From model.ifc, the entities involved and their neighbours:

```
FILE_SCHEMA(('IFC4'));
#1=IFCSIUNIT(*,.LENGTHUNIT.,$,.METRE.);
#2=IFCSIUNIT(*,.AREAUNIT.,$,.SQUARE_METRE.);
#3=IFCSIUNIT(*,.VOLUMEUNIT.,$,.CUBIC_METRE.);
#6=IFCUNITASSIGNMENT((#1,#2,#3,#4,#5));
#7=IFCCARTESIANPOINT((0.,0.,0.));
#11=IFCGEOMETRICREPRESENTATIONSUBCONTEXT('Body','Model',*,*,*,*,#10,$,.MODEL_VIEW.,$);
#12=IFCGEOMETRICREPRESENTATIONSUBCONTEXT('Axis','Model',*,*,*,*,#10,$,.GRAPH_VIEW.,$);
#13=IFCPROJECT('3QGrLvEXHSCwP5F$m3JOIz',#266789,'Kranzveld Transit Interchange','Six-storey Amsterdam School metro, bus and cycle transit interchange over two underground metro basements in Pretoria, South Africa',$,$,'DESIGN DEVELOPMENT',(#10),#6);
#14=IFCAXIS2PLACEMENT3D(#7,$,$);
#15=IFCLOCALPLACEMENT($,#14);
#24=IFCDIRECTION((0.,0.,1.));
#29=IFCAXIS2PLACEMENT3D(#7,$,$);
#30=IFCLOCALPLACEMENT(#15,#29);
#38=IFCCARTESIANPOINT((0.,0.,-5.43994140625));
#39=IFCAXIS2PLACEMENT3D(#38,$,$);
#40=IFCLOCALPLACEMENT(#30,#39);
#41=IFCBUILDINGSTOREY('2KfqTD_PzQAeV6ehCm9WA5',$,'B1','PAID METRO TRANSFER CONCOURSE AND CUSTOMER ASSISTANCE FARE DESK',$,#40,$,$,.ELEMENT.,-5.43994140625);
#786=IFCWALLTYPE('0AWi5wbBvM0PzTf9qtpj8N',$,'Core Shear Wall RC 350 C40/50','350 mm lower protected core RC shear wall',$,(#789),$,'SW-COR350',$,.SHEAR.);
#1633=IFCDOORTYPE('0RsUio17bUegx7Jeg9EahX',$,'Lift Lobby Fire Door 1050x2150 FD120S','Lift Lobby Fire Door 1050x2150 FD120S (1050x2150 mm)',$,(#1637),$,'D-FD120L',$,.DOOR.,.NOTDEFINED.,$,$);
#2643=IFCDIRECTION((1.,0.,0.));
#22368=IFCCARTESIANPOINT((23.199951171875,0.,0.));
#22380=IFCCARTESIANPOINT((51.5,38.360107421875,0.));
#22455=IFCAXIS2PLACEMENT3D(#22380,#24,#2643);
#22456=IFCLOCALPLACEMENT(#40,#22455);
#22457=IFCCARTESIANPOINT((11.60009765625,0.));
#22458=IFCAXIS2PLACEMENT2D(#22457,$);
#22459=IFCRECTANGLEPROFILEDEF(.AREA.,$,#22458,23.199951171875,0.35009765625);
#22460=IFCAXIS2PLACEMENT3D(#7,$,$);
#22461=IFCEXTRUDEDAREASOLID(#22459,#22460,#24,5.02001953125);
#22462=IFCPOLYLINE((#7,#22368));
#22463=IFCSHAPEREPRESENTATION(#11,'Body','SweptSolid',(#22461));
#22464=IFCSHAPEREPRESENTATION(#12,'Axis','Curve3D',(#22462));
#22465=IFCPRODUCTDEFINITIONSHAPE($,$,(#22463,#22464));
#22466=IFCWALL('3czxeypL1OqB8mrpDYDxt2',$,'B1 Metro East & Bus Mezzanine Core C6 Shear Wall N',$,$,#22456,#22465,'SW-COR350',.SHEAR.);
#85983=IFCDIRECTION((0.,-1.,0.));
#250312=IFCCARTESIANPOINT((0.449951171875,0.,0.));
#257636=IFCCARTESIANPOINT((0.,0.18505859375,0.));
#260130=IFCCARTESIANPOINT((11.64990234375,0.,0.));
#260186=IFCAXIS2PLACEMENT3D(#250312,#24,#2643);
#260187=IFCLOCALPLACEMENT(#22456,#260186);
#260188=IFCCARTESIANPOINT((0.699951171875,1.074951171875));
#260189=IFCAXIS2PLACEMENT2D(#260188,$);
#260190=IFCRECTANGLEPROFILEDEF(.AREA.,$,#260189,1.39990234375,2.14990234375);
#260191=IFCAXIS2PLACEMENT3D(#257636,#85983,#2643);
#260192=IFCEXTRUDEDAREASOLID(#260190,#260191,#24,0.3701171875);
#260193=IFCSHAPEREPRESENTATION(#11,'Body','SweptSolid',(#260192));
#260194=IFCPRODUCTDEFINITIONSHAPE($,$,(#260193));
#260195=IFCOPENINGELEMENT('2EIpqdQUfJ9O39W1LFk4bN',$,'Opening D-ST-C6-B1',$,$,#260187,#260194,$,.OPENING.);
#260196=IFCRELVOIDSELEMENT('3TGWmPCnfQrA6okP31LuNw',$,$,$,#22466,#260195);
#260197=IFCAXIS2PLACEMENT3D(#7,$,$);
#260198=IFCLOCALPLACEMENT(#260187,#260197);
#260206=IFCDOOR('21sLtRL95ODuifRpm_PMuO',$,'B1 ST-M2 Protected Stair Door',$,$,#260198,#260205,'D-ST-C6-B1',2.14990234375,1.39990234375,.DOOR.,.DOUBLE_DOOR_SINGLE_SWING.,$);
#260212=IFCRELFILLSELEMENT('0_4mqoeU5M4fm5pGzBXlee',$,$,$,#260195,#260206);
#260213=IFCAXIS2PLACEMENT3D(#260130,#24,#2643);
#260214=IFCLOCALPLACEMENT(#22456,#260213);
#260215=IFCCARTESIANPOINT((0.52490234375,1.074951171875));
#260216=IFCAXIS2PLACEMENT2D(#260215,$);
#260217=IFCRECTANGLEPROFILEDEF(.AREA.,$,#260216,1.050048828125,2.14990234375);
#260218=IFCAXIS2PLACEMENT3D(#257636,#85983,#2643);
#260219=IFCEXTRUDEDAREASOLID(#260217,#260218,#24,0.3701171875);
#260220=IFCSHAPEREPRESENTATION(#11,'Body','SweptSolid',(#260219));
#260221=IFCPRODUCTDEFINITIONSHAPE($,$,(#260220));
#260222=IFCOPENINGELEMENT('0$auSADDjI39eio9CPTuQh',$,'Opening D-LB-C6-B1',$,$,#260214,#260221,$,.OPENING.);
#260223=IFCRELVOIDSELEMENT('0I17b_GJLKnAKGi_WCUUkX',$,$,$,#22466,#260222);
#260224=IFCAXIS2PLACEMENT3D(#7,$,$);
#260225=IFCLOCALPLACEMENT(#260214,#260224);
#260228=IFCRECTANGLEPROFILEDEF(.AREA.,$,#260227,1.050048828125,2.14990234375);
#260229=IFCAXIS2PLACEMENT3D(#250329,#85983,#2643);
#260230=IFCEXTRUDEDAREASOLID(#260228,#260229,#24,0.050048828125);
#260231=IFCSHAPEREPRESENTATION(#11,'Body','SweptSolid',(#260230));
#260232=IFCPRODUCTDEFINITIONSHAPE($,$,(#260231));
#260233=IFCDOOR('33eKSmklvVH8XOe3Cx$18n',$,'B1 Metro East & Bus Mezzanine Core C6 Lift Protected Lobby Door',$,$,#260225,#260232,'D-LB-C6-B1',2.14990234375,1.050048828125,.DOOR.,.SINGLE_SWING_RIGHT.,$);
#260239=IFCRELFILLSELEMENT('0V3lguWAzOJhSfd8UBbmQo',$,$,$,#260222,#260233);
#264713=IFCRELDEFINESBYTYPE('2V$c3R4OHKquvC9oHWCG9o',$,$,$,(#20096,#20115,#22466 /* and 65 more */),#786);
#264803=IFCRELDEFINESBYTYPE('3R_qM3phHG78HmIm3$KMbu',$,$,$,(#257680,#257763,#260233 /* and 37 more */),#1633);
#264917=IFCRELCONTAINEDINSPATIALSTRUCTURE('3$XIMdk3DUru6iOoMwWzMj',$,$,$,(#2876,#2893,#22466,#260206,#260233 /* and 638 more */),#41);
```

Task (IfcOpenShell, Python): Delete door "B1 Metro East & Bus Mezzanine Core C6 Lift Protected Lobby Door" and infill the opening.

```python
import ifcopenshell
import ifcopenshell.api.feature
import ifcopenshell.api.root
import ifcopenshell.geom
import ifcopenshell.util.shape

model = ifcopenshell.open("model.ifc")
settings = ifcopenshell.geom.settings()


def volume(element):
    """Net volume in cubic metres, openings subtracted."""
    shape = ifcopenshell.geom.create_shape(settings, element)
    return ifcopenshell.util.shape.get_volume(shape.geometry)


door = model.by_guid("33eKSmklvVH8XOe3Cx$18n")
opening = door.FillsVoids[0].RelatingOpeningElement
wall = opening.VoidsElements[0].RelatingBuildingElement
before = volume(wall)

ifcopenshell.api.root.remove_product(model, product=door)
ifcopenshell.api.feature.remove_feature(model, feature=opening)

after = volume(wall)

print(f"wall volume {before:.3f} -> {after:.3f} m3")

model.write("model-out.ifc")
```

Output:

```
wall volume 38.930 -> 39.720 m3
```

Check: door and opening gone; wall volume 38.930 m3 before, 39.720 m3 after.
